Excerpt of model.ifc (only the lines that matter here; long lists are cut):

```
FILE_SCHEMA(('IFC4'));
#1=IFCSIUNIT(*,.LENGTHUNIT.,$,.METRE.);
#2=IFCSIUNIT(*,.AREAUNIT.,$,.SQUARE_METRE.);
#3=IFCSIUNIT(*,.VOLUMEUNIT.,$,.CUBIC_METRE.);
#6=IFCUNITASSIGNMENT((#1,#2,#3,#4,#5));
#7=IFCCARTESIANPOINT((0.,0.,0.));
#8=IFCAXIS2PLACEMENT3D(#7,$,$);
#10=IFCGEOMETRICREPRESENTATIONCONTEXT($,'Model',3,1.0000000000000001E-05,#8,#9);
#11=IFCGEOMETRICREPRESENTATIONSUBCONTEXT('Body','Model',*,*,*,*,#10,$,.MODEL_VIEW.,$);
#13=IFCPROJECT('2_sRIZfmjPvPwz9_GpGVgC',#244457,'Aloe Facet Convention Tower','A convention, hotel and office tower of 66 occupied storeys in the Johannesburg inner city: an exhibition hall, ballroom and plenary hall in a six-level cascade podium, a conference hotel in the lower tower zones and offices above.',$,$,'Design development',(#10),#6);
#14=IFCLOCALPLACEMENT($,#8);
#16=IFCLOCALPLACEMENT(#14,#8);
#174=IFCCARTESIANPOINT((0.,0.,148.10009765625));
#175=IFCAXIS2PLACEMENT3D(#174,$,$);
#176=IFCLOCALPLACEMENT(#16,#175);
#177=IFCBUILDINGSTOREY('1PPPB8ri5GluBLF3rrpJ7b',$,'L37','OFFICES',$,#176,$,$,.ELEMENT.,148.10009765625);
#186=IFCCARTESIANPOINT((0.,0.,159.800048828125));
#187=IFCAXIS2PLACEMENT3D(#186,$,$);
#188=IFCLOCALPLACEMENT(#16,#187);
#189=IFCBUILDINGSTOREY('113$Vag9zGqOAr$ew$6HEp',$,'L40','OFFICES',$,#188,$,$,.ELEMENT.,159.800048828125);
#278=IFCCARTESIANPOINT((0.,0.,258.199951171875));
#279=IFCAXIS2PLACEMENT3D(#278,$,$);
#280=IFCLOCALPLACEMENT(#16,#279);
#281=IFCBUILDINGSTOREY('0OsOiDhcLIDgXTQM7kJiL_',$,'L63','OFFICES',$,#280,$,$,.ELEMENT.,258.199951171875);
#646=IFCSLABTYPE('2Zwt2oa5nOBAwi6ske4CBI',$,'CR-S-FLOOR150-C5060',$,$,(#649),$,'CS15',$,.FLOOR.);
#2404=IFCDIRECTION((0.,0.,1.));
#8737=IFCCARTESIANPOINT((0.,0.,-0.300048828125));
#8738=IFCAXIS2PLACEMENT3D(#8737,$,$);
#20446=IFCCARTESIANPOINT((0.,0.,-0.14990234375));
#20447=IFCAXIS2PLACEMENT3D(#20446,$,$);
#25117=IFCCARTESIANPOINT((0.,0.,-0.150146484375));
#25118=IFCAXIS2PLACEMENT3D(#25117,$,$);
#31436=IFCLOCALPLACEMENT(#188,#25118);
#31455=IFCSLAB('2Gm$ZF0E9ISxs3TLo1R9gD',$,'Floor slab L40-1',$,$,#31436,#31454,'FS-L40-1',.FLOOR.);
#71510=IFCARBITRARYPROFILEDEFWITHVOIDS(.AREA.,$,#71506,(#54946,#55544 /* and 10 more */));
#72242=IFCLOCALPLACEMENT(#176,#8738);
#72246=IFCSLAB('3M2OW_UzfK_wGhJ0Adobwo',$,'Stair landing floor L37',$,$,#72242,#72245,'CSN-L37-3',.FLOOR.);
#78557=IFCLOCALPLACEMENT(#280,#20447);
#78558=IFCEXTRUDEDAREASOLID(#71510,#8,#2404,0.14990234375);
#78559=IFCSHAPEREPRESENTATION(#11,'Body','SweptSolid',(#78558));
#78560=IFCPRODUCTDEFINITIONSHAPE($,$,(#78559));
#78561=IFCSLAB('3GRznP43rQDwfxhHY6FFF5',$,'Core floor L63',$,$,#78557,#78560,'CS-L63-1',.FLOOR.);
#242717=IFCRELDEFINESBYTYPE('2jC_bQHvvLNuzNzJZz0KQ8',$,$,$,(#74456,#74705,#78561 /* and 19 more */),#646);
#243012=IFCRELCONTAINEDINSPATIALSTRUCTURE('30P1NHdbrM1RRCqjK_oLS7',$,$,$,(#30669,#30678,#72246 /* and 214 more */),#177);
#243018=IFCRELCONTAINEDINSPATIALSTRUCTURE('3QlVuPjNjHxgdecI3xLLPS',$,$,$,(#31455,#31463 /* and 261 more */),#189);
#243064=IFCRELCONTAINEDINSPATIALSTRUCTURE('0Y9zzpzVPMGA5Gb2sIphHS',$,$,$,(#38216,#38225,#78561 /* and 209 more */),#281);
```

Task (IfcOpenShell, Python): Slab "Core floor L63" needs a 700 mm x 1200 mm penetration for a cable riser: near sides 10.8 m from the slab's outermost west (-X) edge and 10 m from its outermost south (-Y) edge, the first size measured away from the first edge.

```python
import numpy as np
import ifcopenshell
import ifcopenshell.api.feature
import ifcopenshell.api.geometry
import ifcopenshell.api.root
import ifcopenshell.geom
import ifcopenshell.util.placement
import ifcopenshell.util.representation
import ifcopenshell.util.shape
import ifcopenshell.util.unit

model = ifcopenshell.open("model.ifc")
unit_scale = ifcopenshell.util.unit.calculate_unit_scale(model)
settings = ifcopenshell.geom.settings()


def volume(element):
    """Net volume in cubic metres, openings subtracted."""
    shape = ifcopenshell.geom.create_shape(settings, element)
    return ifcopenshell.util.shape.get_volume(shape.geometry)


slab = model.by_guid("3GRznP43rQDwfxhHY6FFF5")
before = volume(slab)

# Extent in the slab's own axes, in metres. The edges named are its -X and -Y sides.
slab_shape = ifcopenshell.geom.create_shape(settings, slab)
vertices = ifcopenshell.util.shape.get_vertices(slab_shape.geometry)
x_min, y_min, bottom = vertices.min(axis=0)
top = vertices[:, 2].max()

opening = ifcopenshell.api.root.create_entity(model, ifc_class="IfcOpeningElement", name="Cable riser opening", predefined_type="OPENING")
context = ifcopenshell.util.representation.get_context(model, "Model", "Body", "MODEL_VIEW")
width, depth = 0.7, 1.2
outline = [(0.0, 0.0), (width, 0.0), (width, depth), (0.0, depth), (0.0, 0.0)]
# Overshoot both faces by 50 mm so the cut is clean.
shape = ifcopenshell.api.geometry.add_slab_representation(
    model, context=context, depth=top - bottom + 0.1, polyline=outline
)
ifcopenshell.api.geometry.assign_representation(model, product=opening, representation=shape)

matrix = ifcopenshell.util.placement.get_local_placement(slab.ObjectPlacement)
matrix[:, 3] = matrix @ np.append(np.array([x_min + 10.8, y_min + 10, bottom - 0.05]) / unit_scale, 1.0)
ifcopenshell.api.geometry.edit_object_placement(model, product=opening, matrix=matrix, is_si=False)
ifcopenshell.api.feature.add_feature(model, feature=opening, element=slab)

after = volume(slab)

print(f"slab volume {before:.3f} -> {after:.3f} m3")

model.write("model_v2.ifc")
```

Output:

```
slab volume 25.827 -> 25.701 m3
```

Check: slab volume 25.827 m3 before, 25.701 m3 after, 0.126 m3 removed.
